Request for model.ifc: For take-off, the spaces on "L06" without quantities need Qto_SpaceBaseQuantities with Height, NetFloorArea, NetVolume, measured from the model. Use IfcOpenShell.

First a look at what the model holds.

```python
import ifcopenshell
import ifcopenshell.util.element
import ifcopenshell.util.unit

model = ifcopenshell.open("model.ifc")
print(model.schema)
for unit_type in ("LENGTHUNIT", "AREAUNIT", "VOLUMEUNIT"):
    print(unit_type, ifcopenshell.util.unit.calculate_unit_scale(model, unit_type))
storey = next(s for s in model.by_type("IfcBuildingStorey") if s.Name == "L06")
spaces = [e for e in ifcopenshell.util.element.get_decomposition(storey) if e.is_a("IfcSpace")]
for e in sorted(spaces, key=lambda e: e.id()):
    print(e.id(), e.is_a(), e.Name, list(ifcopenshell.util.element.get_psets(e, qtos_only=True)), sep=" | ")
```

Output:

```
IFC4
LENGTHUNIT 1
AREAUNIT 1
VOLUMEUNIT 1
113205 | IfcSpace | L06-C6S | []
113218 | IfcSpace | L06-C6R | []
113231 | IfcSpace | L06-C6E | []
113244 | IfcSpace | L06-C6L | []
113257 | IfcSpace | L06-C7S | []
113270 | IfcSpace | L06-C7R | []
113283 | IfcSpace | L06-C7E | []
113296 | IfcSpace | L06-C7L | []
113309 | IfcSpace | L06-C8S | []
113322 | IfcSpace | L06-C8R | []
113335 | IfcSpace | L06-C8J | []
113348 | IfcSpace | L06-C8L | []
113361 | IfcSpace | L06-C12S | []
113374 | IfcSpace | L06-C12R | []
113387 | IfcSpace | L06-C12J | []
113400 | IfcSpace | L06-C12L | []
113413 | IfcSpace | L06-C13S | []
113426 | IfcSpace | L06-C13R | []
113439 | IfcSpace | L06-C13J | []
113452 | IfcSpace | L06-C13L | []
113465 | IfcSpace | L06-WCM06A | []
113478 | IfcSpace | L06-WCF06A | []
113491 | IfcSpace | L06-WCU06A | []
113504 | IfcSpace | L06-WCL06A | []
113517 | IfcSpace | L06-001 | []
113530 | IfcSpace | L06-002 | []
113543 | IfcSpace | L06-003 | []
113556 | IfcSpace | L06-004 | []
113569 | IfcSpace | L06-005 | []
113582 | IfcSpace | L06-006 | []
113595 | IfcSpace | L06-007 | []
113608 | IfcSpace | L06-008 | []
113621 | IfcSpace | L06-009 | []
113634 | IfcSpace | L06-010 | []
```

```python
import ifcopenshell
import ifcopenshell.api.pset
import ifcopenshell.geom
import ifcopenshell.util.element
import ifcopenshell.util.shape
import ifcopenshell.util.unit

model = ifcopenshell.open("model.ifc")
unit_scale = ifcopenshell.util.unit.calculate_unit_scale(model)
area_scale = ifcopenshell.util.unit.calculate_unit_scale(model, "AREAUNIT")
volume_scale = ifcopenshell.util.unit.calculate_unit_scale(model, "VOLUMEUNIT")
settings = ifcopenshell.geom.settings()

storey = next(s for s in model.by_type("IfcBuildingStorey") if s.Name == "L06")
spaces = [e for e in ifcopenshell.util.element.get_decomposition(storey) if e.is_a("IfcSpace")]

for e in sorted(spaces, key=lambda e: e.id()):
    if ifcopenshell.util.element.get_psets(e, qtos_only=True, should_inherit=False):
        continue
    # Geometry comes back in metres, in the element's own axes.
    shape = ifcopenshell.geom.create_shape(settings, e)
    values = {
        "Height": ifcopenshell.util.shape.get_z(shape.geometry) / unit_scale,
        "NetFloorArea": ifcopenshell.util.shape.get_footprint_area(shape.geometry) / area_scale,
        "NetVolume": ifcopenshell.util.shape.get_volume(shape.geometry) / volume_scale,
    }
    qto = ifcopenshell.api.pset.add_qto(model, product=e, name="Qto_SpaceBaseQuantities")
    ifcopenshell.api.pset.edit_qto(model, qto=qto, properties=values)
    print(e.id(), {k: round(v, 3) for k, v in values.items()})

model.write("model_rev.ifc")
```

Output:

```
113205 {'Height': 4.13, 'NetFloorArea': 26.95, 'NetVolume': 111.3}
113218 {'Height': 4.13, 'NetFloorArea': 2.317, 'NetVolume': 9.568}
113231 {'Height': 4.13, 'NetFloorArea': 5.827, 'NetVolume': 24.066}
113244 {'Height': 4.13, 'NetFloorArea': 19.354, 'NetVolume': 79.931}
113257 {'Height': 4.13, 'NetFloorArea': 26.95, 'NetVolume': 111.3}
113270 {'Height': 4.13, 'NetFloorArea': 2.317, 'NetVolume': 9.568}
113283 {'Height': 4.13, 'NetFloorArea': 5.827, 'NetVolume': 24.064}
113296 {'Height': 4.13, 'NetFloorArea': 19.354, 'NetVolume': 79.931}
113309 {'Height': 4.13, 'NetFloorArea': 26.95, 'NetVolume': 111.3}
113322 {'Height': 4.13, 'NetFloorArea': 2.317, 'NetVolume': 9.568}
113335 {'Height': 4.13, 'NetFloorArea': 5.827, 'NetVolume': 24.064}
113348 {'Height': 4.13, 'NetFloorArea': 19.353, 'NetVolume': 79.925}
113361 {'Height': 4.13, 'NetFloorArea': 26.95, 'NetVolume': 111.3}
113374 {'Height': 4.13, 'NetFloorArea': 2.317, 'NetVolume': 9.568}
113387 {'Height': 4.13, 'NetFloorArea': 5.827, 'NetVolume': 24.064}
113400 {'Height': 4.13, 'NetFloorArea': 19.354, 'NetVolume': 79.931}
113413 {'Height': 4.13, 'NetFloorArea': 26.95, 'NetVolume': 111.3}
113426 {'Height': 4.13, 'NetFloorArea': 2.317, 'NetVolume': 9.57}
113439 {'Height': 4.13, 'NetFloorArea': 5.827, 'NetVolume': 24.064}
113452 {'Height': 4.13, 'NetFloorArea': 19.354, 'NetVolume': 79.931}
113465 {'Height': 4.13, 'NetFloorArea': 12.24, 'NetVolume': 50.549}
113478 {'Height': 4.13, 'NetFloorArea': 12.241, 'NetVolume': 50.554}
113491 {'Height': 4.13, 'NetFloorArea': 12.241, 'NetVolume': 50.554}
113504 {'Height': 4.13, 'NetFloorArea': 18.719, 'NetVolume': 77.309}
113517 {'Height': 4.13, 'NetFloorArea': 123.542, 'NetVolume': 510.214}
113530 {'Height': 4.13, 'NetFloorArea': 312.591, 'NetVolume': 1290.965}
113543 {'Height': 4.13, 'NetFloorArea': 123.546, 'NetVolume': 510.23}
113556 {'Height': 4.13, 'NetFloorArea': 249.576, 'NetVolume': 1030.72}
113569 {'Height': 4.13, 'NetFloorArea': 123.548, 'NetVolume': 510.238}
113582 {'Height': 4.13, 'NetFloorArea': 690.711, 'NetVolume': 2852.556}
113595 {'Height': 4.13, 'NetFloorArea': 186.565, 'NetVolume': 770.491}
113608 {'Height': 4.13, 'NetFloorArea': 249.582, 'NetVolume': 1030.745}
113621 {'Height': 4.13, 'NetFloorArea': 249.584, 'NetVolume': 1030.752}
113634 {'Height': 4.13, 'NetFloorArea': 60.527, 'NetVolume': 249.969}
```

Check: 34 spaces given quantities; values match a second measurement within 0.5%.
